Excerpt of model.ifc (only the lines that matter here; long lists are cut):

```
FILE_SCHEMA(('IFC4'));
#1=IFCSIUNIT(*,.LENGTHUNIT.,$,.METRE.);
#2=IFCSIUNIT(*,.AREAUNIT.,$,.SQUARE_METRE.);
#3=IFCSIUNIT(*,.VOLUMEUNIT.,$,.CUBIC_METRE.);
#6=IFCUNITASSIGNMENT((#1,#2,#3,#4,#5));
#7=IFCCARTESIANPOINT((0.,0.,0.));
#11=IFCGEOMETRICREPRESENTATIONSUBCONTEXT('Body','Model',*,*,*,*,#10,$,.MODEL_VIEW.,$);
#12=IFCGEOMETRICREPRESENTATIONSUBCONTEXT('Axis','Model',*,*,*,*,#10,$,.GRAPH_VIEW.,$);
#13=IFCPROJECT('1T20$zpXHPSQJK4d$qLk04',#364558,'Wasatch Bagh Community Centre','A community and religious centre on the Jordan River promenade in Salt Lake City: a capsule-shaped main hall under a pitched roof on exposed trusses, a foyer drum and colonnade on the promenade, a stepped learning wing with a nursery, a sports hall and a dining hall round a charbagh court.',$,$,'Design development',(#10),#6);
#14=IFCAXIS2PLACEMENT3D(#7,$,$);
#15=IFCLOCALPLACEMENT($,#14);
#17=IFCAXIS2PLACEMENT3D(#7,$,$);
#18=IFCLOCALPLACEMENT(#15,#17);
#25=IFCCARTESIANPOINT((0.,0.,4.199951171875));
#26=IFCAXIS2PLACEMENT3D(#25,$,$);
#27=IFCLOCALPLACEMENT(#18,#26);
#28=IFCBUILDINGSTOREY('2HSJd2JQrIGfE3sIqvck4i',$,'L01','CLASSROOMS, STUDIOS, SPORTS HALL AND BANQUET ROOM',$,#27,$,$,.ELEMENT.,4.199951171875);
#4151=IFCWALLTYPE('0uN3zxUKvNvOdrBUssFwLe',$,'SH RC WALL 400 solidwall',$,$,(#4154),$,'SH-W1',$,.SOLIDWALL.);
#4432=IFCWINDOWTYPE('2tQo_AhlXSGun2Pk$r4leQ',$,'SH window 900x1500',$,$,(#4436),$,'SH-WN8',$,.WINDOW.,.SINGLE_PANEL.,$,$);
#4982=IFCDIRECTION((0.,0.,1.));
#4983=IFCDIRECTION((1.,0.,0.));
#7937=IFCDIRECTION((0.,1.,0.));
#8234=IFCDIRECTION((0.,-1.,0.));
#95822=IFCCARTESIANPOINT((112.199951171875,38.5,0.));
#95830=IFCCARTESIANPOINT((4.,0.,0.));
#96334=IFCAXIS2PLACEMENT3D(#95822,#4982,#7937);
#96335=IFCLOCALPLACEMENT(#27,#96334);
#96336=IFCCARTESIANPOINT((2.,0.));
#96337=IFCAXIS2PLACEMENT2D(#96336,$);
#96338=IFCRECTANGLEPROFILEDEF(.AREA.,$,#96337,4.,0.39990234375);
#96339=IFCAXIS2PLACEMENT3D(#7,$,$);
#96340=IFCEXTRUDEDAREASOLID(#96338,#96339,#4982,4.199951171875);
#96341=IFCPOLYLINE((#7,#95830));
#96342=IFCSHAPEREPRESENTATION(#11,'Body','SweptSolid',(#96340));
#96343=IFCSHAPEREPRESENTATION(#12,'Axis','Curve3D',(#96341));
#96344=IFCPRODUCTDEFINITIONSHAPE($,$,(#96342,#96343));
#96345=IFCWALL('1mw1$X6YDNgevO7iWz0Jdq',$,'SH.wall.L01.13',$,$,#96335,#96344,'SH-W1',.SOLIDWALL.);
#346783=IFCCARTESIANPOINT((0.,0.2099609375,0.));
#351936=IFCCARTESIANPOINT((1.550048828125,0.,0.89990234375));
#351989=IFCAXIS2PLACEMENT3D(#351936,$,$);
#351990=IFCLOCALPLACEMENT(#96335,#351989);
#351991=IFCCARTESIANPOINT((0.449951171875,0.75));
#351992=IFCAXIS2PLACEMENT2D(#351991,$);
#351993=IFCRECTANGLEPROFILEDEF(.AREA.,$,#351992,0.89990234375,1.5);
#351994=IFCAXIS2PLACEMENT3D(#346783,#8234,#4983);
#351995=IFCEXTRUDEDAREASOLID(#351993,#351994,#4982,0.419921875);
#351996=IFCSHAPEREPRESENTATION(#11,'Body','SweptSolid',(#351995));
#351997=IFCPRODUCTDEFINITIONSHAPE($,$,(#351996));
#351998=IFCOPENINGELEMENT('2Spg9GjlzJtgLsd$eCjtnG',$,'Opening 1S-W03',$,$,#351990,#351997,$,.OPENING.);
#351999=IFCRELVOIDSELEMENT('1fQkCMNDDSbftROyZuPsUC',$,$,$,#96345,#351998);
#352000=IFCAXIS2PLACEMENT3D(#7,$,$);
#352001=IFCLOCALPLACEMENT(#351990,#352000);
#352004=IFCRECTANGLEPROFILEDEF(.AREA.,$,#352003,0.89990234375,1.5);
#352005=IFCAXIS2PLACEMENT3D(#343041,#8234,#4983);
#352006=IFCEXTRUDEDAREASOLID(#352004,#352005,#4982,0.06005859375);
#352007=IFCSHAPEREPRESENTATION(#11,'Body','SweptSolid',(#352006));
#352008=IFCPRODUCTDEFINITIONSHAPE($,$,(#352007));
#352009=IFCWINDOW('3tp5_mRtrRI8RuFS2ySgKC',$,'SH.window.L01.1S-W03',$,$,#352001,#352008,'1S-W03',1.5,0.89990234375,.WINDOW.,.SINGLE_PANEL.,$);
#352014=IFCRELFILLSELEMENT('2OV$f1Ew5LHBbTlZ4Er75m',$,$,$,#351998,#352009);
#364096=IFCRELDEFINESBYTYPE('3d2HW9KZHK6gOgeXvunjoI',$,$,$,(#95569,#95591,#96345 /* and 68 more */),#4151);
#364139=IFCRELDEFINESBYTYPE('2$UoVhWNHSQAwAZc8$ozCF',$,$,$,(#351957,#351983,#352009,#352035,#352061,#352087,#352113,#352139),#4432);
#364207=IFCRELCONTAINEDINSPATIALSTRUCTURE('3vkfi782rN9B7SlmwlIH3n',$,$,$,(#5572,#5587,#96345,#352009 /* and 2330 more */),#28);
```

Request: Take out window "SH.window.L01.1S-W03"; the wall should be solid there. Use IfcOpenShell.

```python
import ifcopenshell
import ifcopenshell.api.feature
import ifcopenshell.api.root
import ifcopenshell.geom
import ifcopenshell.util.shape

model = ifcopenshell.open("model.ifc")
settings = ifcopenshell.geom.settings()


def volume(element):
    """Net volume in cubic metres, openings subtracted."""
    shape = ifcopenshell.geom.create_shape(settings, element)
    return ifcopenshell.util.shape.get_volume(shape.geometry)


window = model.by_id(352009)
opening = window.FillsVoids[0].RelatingOpeningElement
wall = opening.VoidsElements[0].RelatingBuildingElement
before = volume(wall)

ifcopenshell.api.root.remove_product(model, product=window)
ifcopenshell.api.feature.remove_feature(model, feature=opening)

after = volume(wall)

print(f"wall volume {before:.3f} -> {after:.3f} m3")

model.write("model_v2.ifc")
```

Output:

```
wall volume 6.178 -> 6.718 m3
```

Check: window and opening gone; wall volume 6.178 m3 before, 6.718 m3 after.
